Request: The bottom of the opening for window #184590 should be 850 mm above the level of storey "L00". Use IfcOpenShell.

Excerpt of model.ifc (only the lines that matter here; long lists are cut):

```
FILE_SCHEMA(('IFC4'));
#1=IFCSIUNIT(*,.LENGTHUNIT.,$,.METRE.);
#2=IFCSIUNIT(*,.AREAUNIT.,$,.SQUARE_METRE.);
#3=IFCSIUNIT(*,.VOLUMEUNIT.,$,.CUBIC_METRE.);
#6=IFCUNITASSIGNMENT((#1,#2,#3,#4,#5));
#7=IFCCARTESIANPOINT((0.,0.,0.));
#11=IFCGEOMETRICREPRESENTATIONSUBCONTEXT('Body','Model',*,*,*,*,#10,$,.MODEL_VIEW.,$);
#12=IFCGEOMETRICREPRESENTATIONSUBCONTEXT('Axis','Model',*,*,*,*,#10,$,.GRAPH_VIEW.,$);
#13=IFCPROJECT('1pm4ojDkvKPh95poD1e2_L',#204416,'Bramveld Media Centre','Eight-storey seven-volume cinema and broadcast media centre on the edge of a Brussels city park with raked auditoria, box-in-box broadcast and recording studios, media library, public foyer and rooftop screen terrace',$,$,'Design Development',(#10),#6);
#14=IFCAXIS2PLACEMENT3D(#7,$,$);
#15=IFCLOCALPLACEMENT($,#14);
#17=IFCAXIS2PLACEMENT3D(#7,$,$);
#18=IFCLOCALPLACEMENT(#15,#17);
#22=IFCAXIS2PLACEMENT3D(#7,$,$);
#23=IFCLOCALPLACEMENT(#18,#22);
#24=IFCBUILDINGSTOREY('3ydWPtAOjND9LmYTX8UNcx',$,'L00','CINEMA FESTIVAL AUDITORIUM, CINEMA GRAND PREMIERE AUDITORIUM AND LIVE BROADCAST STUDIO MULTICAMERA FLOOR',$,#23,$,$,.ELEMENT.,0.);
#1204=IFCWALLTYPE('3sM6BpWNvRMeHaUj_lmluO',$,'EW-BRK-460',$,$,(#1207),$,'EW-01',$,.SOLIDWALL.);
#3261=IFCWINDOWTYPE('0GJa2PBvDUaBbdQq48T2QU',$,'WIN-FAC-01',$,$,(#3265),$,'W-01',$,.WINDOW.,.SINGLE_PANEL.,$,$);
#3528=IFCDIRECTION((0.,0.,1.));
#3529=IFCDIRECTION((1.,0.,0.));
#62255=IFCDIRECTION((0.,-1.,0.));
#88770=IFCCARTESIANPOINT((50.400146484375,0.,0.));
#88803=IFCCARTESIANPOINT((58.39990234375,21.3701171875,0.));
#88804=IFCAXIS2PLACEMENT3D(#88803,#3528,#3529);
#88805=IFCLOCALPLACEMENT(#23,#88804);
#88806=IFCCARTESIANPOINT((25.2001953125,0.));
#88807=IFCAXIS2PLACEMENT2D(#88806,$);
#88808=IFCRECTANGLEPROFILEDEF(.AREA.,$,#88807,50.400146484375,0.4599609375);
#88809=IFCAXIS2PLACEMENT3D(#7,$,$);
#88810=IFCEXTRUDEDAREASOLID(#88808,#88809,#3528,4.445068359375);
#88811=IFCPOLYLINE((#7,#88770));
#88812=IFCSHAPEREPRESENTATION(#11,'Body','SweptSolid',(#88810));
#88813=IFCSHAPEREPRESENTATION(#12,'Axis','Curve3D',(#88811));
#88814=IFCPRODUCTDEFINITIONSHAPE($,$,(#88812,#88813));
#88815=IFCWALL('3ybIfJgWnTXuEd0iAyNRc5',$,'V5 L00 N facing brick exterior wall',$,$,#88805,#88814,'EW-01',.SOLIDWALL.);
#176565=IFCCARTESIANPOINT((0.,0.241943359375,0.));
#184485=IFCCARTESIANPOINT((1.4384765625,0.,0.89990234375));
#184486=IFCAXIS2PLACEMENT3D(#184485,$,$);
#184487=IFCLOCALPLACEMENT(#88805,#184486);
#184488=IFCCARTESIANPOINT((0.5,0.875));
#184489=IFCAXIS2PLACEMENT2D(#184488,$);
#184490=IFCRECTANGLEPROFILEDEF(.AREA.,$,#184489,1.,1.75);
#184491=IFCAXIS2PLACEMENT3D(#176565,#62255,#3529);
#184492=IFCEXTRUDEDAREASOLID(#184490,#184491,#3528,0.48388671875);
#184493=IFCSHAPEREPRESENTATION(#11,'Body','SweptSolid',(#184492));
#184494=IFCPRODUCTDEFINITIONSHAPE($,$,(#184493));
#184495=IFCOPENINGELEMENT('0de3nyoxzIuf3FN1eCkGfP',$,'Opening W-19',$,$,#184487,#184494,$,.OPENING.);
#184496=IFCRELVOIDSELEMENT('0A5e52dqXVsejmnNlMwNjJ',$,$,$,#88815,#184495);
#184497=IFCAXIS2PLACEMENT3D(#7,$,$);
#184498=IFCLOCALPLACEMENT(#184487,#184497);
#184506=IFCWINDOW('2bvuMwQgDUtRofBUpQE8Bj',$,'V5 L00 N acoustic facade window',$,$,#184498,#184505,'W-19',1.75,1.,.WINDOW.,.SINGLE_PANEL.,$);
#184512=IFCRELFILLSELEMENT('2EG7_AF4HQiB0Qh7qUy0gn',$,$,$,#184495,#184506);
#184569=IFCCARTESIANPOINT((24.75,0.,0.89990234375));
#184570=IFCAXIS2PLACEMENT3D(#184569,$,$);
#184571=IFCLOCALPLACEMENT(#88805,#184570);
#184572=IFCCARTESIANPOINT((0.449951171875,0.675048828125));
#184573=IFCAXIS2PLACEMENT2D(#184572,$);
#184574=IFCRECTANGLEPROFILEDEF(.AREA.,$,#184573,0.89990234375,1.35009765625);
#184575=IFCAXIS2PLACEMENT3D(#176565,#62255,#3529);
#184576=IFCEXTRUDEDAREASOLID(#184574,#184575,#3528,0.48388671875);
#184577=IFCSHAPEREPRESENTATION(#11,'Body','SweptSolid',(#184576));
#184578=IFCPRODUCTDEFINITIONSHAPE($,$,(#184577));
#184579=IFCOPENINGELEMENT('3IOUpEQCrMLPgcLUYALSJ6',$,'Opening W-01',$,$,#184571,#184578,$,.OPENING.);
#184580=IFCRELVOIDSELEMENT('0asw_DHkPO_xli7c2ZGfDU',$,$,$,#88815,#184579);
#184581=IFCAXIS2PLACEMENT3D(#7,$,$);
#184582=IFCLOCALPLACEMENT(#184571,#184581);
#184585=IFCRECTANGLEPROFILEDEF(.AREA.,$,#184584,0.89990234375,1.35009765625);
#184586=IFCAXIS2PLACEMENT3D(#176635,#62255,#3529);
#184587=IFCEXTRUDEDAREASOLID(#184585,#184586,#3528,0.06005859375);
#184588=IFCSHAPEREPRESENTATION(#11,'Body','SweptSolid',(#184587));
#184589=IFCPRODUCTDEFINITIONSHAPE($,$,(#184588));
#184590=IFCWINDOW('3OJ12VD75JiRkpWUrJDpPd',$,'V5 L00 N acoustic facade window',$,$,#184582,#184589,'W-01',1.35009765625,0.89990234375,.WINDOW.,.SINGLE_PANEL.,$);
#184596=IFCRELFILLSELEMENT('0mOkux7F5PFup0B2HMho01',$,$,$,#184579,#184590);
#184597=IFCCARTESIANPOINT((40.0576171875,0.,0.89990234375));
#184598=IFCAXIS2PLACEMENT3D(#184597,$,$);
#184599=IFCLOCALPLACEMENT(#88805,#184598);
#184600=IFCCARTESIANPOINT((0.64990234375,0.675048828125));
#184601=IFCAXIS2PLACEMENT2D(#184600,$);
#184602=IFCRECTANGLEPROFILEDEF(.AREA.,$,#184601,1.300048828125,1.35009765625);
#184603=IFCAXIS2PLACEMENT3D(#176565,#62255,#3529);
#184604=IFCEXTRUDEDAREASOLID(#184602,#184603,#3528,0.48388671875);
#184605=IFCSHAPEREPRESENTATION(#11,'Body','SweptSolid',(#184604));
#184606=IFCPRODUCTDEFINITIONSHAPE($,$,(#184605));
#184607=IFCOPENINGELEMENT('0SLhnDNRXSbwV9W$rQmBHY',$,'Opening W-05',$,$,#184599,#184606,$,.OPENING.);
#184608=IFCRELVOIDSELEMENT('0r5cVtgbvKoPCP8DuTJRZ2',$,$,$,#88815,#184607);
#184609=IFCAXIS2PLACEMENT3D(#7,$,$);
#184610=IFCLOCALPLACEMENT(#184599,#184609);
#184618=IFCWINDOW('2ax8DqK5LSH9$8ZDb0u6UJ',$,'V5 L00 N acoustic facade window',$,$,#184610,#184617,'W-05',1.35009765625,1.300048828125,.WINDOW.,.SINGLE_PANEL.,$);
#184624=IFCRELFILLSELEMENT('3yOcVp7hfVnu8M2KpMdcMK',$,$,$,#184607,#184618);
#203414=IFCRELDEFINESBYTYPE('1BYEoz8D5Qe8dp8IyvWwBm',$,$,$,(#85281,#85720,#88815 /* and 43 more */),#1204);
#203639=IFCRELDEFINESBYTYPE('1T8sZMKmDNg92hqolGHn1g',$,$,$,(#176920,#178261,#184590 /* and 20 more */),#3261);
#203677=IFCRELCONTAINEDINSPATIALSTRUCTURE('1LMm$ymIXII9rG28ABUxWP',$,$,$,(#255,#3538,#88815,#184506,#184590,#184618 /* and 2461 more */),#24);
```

```python
import numpy as np
import ifcopenshell
import ifcopenshell.api.geometry
import ifcopenshell.geom
import ifcopenshell.util.element
import ifcopenshell.util.placement
import ifcopenshell.util.shape
import ifcopenshell.util.unit

model = ifcopenshell.open("model.ifc")
unit_scale = ifcopenshell.util.unit.calculate_unit_scale(model)

window = model.by_guid("3OJ12VD75JiRkpWUrJDpPd")
opening = window.FillsVoids[0].RelatingOpeningElement
storey = ifcopenshell.util.element.get_container(window, ifc_class="IfcBuildingStorey")
level = ifcopenshell.util.placement.get_local_placement(storey.ObjectPlacement)[2, 3]

# The opening's origin need not be at the sill, so measure its lowest point.
shape = ifcopenshell.geom.create_shape(ifcopenshell.geom.settings(), opening)
bottom = ifcopenshell.util.shape.get_shape_bottom_elevation(shape, shape.geometry) / unit_scale
dz = level + 0.85 - bottom

shift = np.array([0.0, 0.0, dz])
# The window is placed relative to its opening, so it follows when the opening moves.
matrix = ifcopenshell.util.placement.get_local_placement(opening.ObjectPlacement)
matrix[:3, 3] += shift
ifcopenshell.api.geometry.edit_object_placement(
    model, product=opening, matrix=matrix, is_si=False, should_transform_children=True
)

print(f"moved by {dz * unit_scale:+.3f} m")

model.write("model_v2.ifc")
```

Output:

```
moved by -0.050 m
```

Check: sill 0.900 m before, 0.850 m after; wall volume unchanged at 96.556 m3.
